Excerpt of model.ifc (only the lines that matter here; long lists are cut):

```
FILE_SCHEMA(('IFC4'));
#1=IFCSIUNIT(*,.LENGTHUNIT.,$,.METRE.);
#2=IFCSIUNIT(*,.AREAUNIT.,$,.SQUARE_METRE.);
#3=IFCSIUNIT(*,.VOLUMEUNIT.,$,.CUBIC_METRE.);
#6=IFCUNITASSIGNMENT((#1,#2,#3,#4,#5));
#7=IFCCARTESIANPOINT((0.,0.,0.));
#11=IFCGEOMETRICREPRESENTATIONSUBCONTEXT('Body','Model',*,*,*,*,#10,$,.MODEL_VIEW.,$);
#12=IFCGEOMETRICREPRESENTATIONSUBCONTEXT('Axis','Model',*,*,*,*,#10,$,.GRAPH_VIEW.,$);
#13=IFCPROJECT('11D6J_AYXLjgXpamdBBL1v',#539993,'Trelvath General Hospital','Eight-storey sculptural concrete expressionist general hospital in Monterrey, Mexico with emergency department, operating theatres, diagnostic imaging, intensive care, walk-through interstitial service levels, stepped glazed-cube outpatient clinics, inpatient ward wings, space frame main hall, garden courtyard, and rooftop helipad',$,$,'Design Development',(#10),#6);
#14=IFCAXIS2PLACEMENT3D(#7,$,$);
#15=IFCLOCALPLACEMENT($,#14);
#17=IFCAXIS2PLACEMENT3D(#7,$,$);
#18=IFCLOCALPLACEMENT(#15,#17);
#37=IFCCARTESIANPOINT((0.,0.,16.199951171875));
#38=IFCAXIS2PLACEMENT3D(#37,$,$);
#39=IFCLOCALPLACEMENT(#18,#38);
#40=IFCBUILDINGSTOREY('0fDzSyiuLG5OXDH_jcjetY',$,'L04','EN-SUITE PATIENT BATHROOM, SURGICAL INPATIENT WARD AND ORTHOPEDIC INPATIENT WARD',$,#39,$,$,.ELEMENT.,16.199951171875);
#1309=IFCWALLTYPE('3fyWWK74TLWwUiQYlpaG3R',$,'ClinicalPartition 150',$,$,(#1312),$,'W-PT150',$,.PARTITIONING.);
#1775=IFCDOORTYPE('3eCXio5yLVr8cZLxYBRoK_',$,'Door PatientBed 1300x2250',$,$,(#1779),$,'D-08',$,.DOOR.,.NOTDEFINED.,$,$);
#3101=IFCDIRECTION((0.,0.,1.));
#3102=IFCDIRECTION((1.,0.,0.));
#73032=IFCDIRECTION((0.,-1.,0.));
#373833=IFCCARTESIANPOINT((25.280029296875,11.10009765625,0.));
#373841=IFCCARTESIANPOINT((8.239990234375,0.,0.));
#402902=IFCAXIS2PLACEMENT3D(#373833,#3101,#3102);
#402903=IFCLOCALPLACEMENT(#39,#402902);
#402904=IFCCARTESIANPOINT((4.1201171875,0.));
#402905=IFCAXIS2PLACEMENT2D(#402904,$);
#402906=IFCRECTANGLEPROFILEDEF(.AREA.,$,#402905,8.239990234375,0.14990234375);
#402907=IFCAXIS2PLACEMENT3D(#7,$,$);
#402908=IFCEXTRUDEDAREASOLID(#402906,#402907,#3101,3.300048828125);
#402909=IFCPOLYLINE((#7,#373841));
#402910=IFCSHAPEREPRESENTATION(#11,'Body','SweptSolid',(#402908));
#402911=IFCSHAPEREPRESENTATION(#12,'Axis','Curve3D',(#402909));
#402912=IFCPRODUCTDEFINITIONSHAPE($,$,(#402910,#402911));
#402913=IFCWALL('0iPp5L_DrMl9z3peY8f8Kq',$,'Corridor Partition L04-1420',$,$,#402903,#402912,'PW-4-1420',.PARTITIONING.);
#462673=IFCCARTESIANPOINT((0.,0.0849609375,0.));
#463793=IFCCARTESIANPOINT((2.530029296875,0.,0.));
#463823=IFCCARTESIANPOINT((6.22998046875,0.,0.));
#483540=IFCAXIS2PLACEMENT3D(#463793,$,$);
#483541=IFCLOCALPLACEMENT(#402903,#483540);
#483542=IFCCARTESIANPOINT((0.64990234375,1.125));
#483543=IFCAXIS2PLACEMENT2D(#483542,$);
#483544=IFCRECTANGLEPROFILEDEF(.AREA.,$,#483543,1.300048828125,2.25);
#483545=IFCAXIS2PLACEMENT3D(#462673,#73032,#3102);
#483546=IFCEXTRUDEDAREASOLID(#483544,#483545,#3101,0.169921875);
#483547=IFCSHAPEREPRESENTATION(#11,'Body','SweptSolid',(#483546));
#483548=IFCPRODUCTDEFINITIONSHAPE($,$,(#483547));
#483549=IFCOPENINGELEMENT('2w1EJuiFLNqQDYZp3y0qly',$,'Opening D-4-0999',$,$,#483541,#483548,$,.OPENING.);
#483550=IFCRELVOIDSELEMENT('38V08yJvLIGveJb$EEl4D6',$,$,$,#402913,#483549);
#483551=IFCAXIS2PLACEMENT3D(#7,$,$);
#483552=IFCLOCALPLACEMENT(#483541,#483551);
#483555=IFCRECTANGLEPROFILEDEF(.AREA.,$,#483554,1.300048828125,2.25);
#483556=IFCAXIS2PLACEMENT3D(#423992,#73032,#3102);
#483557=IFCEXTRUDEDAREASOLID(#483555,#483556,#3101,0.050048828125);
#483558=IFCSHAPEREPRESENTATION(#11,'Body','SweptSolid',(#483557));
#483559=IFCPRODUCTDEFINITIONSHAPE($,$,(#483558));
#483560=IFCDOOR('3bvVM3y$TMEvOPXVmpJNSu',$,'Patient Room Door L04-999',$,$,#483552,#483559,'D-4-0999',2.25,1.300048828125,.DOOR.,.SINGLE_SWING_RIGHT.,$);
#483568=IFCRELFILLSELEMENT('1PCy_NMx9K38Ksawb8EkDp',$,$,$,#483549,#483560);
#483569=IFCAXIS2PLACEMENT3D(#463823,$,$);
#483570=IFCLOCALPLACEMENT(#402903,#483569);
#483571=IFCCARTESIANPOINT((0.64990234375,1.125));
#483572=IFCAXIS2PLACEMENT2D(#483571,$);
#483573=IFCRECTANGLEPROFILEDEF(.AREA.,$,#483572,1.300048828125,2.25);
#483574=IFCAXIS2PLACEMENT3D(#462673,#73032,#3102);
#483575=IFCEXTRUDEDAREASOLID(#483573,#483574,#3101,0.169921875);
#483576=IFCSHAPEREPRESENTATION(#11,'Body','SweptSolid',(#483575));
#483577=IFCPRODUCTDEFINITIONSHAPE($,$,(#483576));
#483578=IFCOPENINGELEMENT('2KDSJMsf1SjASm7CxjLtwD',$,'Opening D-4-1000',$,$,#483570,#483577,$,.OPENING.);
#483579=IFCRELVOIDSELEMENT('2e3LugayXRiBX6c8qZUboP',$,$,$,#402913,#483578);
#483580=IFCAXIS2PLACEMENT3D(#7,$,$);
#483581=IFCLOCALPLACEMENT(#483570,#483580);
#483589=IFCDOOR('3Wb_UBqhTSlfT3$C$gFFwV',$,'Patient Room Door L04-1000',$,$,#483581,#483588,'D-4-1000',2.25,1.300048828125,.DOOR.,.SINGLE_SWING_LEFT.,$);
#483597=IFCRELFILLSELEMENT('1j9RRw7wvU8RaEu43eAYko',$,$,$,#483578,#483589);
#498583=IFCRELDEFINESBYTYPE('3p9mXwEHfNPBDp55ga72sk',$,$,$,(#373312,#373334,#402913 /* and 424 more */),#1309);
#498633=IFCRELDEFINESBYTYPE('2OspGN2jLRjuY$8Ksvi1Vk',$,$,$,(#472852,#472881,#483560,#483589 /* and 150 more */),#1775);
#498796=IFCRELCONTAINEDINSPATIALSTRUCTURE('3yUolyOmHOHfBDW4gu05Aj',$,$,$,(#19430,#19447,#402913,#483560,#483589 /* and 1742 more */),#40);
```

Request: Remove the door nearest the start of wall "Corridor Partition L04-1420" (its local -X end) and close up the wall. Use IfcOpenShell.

```python
import ifcopenshell
import ifcopenshell.api.feature
import ifcopenshell.api.root
import ifcopenshell.geom
import ifcopenshell.util.shape

model = ifcopenshell.open("model.ifc")
settings = ifcopenshell.geom.settings()


def volume(element):
    """Net volume in cubic metres, openings subtracted."""
    shape = ifcopenshell.geom.create_shape(settings, element)
    return ifcopenshell.util.shape.get_volume(shape.geometry)


door = model.by_id(483560)
opening = door.FillsVoids[0].RelatingOpeningElement
wall = opening.VoidsElements[0].RelatingBuildingElement
before = volume(wall)

ifcopenshell.api.root.remove_product(model, product=door)
ifcopenshell.api.feature.remove_feature(model, feature=opening)

after = volume(wall)

print(f"wall volume {before:.3f} -> {after:.3f} m3")

model.write("model-out.ifc")
```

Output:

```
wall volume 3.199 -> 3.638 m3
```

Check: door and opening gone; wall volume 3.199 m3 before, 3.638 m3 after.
